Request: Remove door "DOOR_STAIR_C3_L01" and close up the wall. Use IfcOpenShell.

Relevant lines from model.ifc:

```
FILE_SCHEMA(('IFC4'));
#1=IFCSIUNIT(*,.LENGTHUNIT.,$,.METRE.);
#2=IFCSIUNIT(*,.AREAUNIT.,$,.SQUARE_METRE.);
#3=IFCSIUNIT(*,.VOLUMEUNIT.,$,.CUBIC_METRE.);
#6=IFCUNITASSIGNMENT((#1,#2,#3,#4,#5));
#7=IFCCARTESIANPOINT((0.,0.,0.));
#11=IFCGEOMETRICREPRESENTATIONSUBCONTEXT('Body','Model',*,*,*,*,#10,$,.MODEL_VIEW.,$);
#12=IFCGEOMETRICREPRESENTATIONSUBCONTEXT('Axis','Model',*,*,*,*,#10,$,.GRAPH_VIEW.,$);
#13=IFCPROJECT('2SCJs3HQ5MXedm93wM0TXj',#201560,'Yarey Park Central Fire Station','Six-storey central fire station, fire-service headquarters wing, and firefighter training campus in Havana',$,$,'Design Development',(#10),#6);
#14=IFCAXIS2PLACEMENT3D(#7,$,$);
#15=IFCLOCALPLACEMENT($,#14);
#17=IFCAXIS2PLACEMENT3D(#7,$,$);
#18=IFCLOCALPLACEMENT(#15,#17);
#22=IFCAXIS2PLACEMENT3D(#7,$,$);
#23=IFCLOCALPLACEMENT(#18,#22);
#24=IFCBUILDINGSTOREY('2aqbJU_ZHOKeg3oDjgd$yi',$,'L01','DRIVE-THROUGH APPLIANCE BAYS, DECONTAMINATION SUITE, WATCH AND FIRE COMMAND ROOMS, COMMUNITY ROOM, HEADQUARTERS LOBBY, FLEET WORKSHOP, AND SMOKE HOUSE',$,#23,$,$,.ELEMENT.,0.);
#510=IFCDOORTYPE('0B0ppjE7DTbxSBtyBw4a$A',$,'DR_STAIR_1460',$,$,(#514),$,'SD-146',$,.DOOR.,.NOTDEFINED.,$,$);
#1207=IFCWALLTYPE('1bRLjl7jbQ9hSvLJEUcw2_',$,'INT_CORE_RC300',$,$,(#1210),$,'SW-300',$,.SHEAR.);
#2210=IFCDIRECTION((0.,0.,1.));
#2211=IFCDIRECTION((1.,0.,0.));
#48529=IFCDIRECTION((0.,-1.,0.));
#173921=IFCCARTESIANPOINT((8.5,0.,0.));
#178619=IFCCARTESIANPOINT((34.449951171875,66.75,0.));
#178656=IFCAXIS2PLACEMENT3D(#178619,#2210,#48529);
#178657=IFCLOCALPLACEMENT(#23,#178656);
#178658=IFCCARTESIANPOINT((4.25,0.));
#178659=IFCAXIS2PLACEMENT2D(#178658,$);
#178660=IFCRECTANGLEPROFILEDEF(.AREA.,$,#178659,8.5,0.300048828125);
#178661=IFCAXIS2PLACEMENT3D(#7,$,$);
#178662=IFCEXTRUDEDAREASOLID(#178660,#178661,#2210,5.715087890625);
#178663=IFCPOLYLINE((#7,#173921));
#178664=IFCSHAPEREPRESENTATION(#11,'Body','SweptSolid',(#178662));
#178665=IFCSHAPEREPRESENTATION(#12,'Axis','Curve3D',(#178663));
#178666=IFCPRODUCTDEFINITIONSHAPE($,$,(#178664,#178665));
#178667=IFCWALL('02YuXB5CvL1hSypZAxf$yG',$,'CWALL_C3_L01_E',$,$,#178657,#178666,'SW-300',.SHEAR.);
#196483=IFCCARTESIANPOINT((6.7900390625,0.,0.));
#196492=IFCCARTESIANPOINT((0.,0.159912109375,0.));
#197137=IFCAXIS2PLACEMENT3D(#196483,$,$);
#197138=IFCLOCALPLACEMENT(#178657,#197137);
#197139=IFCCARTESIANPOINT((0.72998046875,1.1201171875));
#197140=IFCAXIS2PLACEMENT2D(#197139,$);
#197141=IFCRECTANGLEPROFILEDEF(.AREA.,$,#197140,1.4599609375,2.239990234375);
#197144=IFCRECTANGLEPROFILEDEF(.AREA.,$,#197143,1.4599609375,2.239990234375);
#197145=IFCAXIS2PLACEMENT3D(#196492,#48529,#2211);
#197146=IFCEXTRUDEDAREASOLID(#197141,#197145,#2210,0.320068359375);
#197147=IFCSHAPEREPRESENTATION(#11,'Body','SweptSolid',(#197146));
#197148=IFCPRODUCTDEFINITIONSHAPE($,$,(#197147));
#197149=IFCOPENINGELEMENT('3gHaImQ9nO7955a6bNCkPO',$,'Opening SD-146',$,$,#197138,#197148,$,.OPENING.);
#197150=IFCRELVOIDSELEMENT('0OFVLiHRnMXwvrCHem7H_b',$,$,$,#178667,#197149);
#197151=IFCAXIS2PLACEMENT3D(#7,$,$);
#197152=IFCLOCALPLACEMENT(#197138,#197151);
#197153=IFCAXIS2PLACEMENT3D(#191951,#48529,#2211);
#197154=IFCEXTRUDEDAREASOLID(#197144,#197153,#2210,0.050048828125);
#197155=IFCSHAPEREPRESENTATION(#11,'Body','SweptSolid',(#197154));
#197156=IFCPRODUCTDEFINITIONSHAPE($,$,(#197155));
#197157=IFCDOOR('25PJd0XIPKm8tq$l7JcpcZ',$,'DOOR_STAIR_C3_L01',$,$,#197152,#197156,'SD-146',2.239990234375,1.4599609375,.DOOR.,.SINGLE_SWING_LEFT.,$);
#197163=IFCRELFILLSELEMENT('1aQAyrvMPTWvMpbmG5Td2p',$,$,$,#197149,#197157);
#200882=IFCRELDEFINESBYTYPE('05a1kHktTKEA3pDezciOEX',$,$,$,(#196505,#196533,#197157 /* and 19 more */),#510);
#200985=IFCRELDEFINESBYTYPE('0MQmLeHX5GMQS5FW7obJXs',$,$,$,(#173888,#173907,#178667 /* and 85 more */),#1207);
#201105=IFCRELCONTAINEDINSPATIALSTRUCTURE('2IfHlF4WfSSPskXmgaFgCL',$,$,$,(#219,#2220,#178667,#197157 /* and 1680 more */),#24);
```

```python
import ifcopenshell
import ifcopenshell.api.feature
import ifcopenshell.api.root
import ifcopenshell.geom
import ifcopenshell.util.shape

model = ifcopenshell.open("model.ifc")
settings = ifcopenshell.geom.settings()


def volume(element):
    """Net volume in cubic metres, openings subtracted."""
    shape = ifcopenshell.geom.create_shape(settings, element)
    return ifcopenshell.util.shape.get_volume(shape.geometry)


door = model.by_guid("25PJd0XIPKm8tq$l7JcpcZ")
opening = door.FillsVoids[0].RelatingOpeningElement
wall = opening.VoidsElements[0].RelatingBuildingElement
before = volume(wall)

ifcopenshell.api.root.remove_product(model, product=door)
ifcopenshell.api.feature.remove_feature(model, feature=opening)

after = volume(wall)

print(f"wall volume {before:.3f} -> {after:.3f} m3")

model.write("model-out.ifc")
```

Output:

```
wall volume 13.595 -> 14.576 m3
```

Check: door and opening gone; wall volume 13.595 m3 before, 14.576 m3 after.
